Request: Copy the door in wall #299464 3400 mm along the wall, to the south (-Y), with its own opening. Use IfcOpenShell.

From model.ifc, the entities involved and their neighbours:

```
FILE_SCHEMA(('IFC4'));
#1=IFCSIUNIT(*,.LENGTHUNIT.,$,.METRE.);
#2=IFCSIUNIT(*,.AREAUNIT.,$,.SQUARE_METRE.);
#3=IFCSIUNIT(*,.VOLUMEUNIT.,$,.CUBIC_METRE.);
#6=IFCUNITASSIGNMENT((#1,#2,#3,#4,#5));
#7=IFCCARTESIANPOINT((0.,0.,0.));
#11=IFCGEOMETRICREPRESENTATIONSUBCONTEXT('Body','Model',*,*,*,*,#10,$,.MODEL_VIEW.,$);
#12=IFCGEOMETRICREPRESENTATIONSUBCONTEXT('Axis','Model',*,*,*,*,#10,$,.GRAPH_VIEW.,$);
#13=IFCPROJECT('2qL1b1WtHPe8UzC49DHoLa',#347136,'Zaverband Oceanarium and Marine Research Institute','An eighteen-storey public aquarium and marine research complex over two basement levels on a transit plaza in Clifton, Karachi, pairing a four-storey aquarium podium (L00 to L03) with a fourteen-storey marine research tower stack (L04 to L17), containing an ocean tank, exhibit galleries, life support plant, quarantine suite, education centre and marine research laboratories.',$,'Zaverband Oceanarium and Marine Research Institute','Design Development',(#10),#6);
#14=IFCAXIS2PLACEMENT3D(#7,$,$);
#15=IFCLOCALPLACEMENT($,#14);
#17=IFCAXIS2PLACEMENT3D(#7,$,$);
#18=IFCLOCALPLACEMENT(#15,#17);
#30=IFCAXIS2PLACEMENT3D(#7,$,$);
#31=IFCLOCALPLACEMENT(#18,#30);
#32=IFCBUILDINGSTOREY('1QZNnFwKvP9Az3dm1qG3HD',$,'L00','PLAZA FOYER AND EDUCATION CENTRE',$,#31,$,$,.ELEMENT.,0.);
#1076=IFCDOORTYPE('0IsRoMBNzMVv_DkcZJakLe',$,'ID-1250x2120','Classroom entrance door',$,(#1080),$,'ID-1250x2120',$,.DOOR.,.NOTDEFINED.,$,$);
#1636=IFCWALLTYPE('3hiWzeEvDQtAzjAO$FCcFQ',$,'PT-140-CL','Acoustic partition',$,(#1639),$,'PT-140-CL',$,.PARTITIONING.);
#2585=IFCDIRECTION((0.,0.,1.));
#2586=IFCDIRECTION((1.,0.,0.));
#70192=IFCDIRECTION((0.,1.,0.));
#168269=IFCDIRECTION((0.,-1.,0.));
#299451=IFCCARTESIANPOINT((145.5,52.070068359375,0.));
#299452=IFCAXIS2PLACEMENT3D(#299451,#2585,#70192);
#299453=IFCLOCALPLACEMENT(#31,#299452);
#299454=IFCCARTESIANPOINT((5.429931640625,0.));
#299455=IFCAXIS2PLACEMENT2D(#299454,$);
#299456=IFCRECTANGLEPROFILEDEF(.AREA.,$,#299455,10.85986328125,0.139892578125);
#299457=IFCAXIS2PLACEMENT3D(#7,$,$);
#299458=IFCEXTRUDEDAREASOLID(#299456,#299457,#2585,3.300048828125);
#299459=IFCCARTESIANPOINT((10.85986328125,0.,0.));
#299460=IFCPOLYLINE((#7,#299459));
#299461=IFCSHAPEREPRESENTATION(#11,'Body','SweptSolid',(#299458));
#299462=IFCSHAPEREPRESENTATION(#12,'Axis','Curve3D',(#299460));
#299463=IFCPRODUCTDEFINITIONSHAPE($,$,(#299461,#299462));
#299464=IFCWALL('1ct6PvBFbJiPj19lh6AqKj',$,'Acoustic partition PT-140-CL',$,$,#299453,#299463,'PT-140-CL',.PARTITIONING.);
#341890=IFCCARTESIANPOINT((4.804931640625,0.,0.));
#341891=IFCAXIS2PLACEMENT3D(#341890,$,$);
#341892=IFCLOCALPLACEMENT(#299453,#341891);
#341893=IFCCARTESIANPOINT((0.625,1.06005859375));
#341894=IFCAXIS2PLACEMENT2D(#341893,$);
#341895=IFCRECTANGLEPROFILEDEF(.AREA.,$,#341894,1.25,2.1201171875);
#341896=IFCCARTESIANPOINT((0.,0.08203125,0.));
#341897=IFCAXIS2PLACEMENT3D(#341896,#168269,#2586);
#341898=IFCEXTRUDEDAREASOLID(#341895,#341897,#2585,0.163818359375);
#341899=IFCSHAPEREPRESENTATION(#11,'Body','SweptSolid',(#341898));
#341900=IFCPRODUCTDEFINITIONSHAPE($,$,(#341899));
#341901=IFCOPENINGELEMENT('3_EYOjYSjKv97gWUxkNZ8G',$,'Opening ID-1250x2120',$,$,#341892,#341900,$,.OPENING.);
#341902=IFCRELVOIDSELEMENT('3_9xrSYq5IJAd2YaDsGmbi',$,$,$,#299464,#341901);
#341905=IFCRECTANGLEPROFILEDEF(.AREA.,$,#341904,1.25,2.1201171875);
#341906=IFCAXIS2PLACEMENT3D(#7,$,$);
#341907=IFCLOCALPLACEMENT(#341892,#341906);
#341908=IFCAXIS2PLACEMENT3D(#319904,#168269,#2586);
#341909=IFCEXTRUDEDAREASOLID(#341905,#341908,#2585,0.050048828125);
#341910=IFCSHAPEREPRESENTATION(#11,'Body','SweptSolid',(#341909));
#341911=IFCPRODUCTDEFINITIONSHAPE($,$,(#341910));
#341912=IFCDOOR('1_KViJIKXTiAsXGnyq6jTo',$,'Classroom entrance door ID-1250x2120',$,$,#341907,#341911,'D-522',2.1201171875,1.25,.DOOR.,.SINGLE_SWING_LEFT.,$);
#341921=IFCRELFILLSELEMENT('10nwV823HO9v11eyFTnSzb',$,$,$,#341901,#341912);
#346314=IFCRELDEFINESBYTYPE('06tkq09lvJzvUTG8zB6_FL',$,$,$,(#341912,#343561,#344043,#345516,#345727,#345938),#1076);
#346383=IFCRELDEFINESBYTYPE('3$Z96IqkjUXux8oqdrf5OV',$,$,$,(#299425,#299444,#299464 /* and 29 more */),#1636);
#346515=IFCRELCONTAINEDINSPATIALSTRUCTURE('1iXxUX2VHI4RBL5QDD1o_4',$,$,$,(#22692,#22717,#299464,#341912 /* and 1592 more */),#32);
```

```python
import ifcopenshell
import ifcopenshell.api.feature
import ifcopenshell.api.geometry
import ifcopenshell.api.root
import ifcopenshell.geom
import ifcopenshell.util.element
import ifcopenshell.util.placement
import ifcopenshell.util.shape
import ifcopenshell.util.unit

model = ifcopenshell.open("model.ifc")
unit_scale = ifcopenshell.util.unit.calculate_unit_scale(model)
settings = ifcopenshell.geom.settings()


def volume(element):
    """Net volume in cubic metres, openings subtracted."""
    shape = ifcopenshell.geom.create_shape(settings, element)
    return ifcopenshell.util.shape.get_volume(shape.geometry)


door = model.by_guid("1_KViJIKXTiAsXGnyq6jTo")
opening = door.FillsVoids[0].RelatingOpeningElement
wall = opening.VoidsElements[0].RelatingBuildingElement
before = volume(wall)
shift = ifcopenshell.util.placement.get_local_placement(wall.ObjectPlacement)[:3, 0] * -3.4 / unit_scale

# copy_class copies the void relationship, type, container and properties, but no geometry.
new_opening = ifcopenshell.api.root.copy_class(model, product=opening)
new_opening.Representation = ifcopenshell.util.element.copy_deep(
    model, opening.Representation, exclude=["IfcGeometricRepresentationContext", "IfcRepresentationMap"]
)
new_door = ifcopenshell.api.root.copy_class(model, product=door)
new_door.Representation = ifcopenshell.util.element.copy_deep(
    model, door.Representation, exclude=["IfcGeometricRepresentationContext", "IfcRepresentationMap"]
)
new_door.Tag = None
ifcopenshell.api.feature.add_filling(model, opening=new_opening, element=new_door)

for old, new in ((opening, new_opening), (door, new_door)):
    matrix = ifcopenshell.util.placement.get_local_placement(old.ObjectPlacement)
    matrix[:3, 3] += shift
    ifcopenshell.api.geometry.edit_object_placement(model, product=new, matrix=matrix, is_si=False)

after = volume(wall)

print(f"wall volume {before:.3f} -> {after:.3f} m3")

model.write("model_v2.ifc")
```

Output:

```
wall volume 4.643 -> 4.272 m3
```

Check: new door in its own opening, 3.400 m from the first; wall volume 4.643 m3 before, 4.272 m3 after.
